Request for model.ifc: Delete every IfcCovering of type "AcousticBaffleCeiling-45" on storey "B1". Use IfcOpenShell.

First a look at what the model holds.

```python
import ifcopenshell
import ifcopenshell.util.element

model = ifcopenshell.open("model.ifc")
print(model.schema)
storey = next(s for s in model.by_type("IfcBuildingStorey") if s.Name == "B1")
coverings = [e for e in ifcopenshell.util.element.get_decomposition(storey) if e.is_a("IfcCovering")]
seen = {}
for e in coverings:
    element_type = ifcopenshell.util.element.get_type(e)
    name = element_type.Name if element_type not in (None, e) else None
    seen[name] = seen.get(name, 0) + 1
for name, count in sorted(seen.items(), key=str):
    print(count, "x", name)
```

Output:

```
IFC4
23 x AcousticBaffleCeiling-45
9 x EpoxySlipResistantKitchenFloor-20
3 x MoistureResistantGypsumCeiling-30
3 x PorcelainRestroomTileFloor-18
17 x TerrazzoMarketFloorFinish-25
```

```python
import ifcopenshell
import ifcopenshell.api.root
import ifcopenshell.util.element

model = ifcopenshell.open("model.ifc")

storey = next(s for s in model.by_type("IfcBuildingStorey") if s.Name == "B1")
coverings = [e for e in ifcopenshell.util.element.get_decomposition(storey) if e.is_a("IfcCovering")]
targets = [e for e in coverings if (t := ifcopenshell.util.element.get_type(e)) not in (None, e) and t.Name == "AcousticBaffleCeiling-45"]

for e in targets:
    ifcopenshell.api.root.remove_product(model, product=e)
print(len(targets), "removed")

model.write("model_rev.ifc")
```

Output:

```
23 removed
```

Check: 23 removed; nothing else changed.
